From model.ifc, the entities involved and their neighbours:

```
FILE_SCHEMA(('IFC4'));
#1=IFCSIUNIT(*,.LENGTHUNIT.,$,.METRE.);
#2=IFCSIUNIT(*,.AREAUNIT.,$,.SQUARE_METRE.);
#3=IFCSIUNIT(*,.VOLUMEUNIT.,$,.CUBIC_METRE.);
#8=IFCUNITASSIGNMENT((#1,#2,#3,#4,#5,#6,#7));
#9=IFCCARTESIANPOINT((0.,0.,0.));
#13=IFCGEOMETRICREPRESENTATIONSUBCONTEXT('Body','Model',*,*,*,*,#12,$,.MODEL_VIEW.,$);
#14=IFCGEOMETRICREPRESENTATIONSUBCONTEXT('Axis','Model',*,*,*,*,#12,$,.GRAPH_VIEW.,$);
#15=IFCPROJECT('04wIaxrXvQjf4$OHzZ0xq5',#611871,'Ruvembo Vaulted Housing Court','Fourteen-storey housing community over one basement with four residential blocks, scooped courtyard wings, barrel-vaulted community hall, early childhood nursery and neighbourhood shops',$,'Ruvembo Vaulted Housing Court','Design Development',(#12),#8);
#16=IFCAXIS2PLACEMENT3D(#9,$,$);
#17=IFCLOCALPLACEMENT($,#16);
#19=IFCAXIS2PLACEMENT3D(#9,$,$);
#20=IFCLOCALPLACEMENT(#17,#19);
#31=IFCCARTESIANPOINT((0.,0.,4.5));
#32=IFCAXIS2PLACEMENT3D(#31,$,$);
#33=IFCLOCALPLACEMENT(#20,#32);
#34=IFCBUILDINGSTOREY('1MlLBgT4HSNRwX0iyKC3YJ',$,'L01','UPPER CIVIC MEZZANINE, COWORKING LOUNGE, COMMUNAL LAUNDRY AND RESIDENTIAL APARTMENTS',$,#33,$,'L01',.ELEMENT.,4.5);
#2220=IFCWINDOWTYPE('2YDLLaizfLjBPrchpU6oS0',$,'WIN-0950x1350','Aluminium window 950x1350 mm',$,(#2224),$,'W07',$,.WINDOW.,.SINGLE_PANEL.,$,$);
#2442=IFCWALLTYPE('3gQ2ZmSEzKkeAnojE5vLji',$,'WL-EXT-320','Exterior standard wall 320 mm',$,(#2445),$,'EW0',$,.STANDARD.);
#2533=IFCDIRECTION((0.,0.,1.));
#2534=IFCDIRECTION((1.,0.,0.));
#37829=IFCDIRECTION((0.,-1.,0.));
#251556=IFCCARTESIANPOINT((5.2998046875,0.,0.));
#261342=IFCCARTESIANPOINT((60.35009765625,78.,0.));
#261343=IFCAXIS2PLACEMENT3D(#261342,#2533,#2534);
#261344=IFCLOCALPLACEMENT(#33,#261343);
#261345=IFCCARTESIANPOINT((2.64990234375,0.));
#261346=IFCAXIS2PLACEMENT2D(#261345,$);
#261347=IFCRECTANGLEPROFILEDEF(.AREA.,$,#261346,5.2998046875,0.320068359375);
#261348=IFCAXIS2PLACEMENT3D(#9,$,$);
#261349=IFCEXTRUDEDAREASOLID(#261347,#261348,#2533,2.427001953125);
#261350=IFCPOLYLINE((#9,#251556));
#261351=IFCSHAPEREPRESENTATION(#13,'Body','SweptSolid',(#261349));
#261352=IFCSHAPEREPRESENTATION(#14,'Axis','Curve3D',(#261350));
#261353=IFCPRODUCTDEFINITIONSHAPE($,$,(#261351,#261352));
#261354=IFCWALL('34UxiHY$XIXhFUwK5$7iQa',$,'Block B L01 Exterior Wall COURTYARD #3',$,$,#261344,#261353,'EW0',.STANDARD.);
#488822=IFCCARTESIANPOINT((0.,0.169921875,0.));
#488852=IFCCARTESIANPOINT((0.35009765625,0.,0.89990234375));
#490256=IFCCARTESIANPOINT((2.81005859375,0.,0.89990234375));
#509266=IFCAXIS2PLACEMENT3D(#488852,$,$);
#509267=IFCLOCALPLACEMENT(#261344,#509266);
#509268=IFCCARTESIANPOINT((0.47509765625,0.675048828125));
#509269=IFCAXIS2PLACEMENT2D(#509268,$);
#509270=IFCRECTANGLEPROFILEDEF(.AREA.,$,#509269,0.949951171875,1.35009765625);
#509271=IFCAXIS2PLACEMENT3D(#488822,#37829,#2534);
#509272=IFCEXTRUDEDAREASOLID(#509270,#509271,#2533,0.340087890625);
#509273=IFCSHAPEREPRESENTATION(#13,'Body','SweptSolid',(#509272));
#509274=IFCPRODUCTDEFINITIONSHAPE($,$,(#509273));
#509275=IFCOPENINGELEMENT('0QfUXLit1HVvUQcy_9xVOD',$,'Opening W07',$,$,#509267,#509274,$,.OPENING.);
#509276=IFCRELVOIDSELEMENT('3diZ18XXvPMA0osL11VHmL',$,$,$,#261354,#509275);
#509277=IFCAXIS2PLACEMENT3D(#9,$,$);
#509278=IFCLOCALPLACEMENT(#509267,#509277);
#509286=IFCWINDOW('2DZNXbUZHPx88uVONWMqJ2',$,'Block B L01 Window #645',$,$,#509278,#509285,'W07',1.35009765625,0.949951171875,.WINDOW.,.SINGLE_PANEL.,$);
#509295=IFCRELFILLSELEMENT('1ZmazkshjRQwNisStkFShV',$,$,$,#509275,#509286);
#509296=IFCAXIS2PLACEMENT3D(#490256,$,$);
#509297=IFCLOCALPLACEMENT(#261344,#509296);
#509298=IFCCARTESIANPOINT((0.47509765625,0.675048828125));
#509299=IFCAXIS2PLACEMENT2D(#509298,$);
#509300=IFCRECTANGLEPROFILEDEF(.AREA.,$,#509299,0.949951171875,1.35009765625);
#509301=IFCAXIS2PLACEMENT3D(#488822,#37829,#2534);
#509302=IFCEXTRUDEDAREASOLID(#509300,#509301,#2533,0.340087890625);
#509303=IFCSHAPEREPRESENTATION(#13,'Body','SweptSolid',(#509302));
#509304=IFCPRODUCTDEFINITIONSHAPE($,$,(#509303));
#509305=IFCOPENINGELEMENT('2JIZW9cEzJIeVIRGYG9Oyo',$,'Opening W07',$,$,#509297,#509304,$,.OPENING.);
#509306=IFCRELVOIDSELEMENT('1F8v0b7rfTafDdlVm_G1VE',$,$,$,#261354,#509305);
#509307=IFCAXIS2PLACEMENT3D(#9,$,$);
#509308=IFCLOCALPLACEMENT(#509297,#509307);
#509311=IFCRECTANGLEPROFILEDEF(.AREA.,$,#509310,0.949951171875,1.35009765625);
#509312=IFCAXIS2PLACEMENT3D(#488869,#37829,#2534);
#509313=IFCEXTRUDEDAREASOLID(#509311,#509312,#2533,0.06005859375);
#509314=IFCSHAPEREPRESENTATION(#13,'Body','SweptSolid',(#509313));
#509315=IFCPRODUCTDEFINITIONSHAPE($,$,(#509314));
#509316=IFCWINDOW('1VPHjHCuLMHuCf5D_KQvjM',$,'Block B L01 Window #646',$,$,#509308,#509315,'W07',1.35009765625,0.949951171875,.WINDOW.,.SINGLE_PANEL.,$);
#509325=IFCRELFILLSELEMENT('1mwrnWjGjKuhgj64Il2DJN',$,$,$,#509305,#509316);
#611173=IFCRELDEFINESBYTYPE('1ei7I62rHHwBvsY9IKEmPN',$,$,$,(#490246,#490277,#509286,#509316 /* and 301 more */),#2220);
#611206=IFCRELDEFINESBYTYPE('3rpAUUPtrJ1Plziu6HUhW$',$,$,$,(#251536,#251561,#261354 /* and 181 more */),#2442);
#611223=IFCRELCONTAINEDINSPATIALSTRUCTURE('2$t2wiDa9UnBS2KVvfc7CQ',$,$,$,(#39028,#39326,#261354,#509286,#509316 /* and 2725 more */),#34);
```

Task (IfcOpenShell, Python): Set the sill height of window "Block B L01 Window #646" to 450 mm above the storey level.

```python
import numpy as np
import ifcopenshell
import ifcopenshell.api.geometry
import ifcopenshell.geom
import ifcopenshell.util.element
import ifcopenshell.util.placement
import ifcopenshell.util.shape
import ifcopenshell.util.unit

model = ifcopenshell.open("model.ifc")
unit_scale = ifcopenshell.util.unit.calculate_unit_scale(model)

window = model.by_guid("1VPHjHCuLMHuCf5D_KQvjM")
opening = window.FillsVoids[0].RelatingOpeningElement
storey = ifcopenshell.util.element.get_container(window, ifc_class="IfcBuildingStorey")
level = ifcopenshell.util.placement.get_local_placement(storey.ObjectPlacement)[2, 3]

# The opening's origin need not be at the sill, so measure its lowest point.
shape = ifcopenshell.geom.create_shape(ifcopenshell.geom.settings(), opening)
bottom = ifcopenshell.util.shape.get_shape_bottom_elevation(shape, shape.geometry) / unit_scale
dz = level + 0.45 / unit_scale - bottom

shift = np.array([0.0, 0.0, dz])
# The window is placed relative to its opening, so it follows when the opening moves.
matrix = ifcopenshell.util.placement.get_local_placement(opening.ObjectPlacement)
matrix[:3, 3] += shift
ifcopenshell.api.geometry.edit_object_placement(
    model, product=opening, matrix=matrix, is_si=False, should_transform_children=True
)

print(f"moved by {dz * unit_scale:+.3f} m")

model.write("model-out.ifc")
```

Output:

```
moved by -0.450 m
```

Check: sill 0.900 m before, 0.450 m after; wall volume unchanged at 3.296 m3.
